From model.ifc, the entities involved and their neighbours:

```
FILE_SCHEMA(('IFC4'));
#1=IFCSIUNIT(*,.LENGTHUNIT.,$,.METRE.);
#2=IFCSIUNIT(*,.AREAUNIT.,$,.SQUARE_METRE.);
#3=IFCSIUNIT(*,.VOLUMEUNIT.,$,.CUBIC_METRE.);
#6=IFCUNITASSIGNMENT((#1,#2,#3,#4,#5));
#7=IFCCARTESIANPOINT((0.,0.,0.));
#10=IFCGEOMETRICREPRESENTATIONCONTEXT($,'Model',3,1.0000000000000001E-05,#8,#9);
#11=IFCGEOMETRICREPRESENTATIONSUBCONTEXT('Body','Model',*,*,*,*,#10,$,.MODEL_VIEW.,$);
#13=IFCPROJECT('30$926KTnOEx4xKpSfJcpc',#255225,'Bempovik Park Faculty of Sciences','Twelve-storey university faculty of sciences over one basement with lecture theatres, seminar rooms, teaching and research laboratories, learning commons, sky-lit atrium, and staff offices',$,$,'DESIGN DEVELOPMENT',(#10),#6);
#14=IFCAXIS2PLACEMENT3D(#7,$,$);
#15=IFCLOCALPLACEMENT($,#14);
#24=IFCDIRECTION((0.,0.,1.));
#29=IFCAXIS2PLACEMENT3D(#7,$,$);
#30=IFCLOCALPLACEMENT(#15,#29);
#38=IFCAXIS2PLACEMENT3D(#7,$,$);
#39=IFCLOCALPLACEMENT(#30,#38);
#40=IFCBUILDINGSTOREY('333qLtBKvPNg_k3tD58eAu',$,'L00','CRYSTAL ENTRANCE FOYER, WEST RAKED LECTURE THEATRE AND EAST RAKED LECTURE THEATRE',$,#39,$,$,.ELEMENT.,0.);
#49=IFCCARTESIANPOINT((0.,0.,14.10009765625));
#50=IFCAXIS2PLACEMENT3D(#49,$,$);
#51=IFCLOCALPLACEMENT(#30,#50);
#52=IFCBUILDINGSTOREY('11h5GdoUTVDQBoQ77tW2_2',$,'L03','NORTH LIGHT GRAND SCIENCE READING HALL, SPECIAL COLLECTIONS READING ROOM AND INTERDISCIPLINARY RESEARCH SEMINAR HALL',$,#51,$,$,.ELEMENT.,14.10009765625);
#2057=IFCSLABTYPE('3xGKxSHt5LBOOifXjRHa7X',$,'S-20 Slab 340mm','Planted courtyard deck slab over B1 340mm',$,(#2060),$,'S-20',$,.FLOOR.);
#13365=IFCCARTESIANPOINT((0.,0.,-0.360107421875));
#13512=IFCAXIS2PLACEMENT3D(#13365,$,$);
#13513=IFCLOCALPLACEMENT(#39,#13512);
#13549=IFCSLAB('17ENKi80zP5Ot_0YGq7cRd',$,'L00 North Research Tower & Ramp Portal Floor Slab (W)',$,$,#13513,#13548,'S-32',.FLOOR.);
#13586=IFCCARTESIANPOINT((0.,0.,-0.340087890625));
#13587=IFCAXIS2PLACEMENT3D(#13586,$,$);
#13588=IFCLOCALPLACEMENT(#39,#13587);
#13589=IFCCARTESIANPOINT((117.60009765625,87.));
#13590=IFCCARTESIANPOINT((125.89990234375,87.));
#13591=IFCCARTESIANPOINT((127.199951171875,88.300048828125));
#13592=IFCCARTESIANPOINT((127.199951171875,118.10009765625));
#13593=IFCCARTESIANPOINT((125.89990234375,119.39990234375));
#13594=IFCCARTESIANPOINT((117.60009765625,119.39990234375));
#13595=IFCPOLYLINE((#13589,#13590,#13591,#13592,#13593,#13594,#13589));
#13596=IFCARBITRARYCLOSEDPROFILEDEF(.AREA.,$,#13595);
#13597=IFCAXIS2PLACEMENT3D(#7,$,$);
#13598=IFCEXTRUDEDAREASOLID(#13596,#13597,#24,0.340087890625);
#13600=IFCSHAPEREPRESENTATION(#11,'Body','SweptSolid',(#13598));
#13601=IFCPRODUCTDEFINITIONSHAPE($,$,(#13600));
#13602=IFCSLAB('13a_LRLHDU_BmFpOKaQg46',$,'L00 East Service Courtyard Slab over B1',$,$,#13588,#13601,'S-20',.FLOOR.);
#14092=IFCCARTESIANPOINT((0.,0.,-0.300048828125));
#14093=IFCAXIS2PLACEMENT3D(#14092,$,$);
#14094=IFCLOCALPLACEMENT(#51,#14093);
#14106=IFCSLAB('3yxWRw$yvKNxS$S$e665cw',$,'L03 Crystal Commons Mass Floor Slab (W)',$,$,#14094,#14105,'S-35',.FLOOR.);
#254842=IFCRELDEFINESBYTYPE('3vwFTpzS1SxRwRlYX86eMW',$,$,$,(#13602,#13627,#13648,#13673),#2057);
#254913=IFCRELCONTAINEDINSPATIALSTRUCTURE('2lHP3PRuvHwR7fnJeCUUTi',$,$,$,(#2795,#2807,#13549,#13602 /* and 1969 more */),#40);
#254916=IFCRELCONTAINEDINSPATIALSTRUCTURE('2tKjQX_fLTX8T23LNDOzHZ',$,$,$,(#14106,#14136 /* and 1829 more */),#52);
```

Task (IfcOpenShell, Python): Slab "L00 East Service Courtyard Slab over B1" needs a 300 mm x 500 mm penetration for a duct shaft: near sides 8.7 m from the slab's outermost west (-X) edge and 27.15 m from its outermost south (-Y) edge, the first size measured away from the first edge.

```python
import numpy as np
import ifcopenshell
import ifcopenshell.api.feature
import ifcopenshell.api.geometry
import ifcopenshell.api.root
import ifcopenshell.geom
import ifcopenshell.util.placement
import ifcopenshell.util.representation
import ifcopenshell.util.shape
import ifcopenshell.util.unit

model = ifcopenshell.open("model.ifc")
unit_scale = ifcopenshell.util.unit.calculate_unit_scale(model)
settings = ifcopenshell.geom.settings()


def volume(element):
    """Net volume in cubic metres, openings subtracted."""
    shape = ifcopenshell.geom.create_shape(settings, element)
    return ifcopenshell.util.shape.get_volume(shape.geometry)


slab = model.by_guid("13a_LRLHDU_BmFpOKaQg46")
before = volume(slab)

# Extent in the slab's own axes, in metres. The edges named are its -X and -Y sides.
slab_shape = ifcopenshell.geom.create_shape(settings, slab)
vertices = ifcopenshell.util.shape.get_vertices(slab_shape.geometry)
x_min, y_min, bottom = vertices.min(axis=0)
top = vertices[:, 2].max()

opening = ifcopenshell.api.root.create_entity(model, ifc_class="IfcOpeningElement", name="Duct shaft opening", predefined_type="OPENING")
context = ifcopenshell.util.representation.get_context(model, "Model", "Body", "MODEL_VIEW")
width, depth = 0.3, 0.5
outline = [(0.0, 0.0), (width, 0.0), (width, depth), (0.0, depth), (0.0, 0.0)]
# Overshoot both faces by 50 mm so the cut is clean.
shape = ifcopenshell.api.geometry.add_slab_representation(
    model, context=context, depth=top - bottom + 0.1, polyline=outline
)
ifcopenshell.api.geometry.assign_representation(model, product=opening, representation=shape)

matrix = ifcopenshell.util.placement.get_local_placement(slab.ObjectPlacement)
matrix[:, 3] = matrix @ np.append(np.array([x_min + 8.7, y_min + 27.15, bottom - 0.05]) / unit_scale, 1.0)
ifcopenshell.api.geometry.edit_object_placement(model, product=opening, matrix=matrix, is_si=False)
ifcopenshell.api.feature.add_feature(model, feature=opening, element=slab)

after = volume(slab)

print(f"slab volume {before:.3f} -> {after:.3f} m3")

model.write("model_rev.ifc")
```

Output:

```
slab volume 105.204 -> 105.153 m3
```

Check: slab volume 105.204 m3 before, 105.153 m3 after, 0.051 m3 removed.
